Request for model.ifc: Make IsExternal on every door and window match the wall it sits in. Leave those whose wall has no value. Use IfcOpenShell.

First a look at what the model holds.

```python
import ifcopenshell
import ifcopenshell.util.element

model = ifcopenshell.open("model.ifc")
print(model.schema)
seen = {}
for e in model.by_type("IfcDoor") + model.by_type("IfcWindow"):
    if not e.FillsVoids:
        continue
    host = e.FillsVoids[0].RelatingOpeningElement.VoidsElements[0].RelatingBuildingElement
    own = ifcopenshell.util.element.get_pset(e, f"Pset_{e.is_a()[3:].removesuffix('StandardCase')}Common", "IsExternal")
    wall = ifcopenshell.util.element.get_pset(host, "Pset_WallCommon", "IsExternal")
    seen[e.is_a(), own, wall] = seen.get((e.is_a(), own, wall), 0) + 1
for (cls, own, wall), count in sorted(seen.items(), key=str):
    print(count, cls, "IsExternal:", own, "| host wall:", wall)
```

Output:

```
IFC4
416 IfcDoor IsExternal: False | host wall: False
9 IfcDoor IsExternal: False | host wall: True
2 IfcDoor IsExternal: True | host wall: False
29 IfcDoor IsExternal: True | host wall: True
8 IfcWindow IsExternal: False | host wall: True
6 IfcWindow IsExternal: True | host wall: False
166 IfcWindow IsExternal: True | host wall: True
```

```python
import ifcopenshell
import ifcopenshell.api.pset
import ifcopenshell.util.element

model = ifcopenshell.open("model.ifc")

count = 0
for ifc_class, pset_name in (("IfcDoor", "Pset_DoorCommon"), ("IfcWindow", "Pset_WindowCommon")):
    for e in model.by_type(ifc_class):
        if not e.FillsVoids:
            continue
        host = e.FillsVoids[0].RelatingOpeningElement.VoidsElements[0].RelatingBuildingElement
        external = ifcopenshell.util.element.get_pset(host, "Pset_WallCommon", "IsExternal")
        if external is None or ifcopenshell.util.element.get_pset(e, pset_name, "IsExternal") == external:
            continue
        pset = ifcopenshell.api.pset.add_pset(model, product=e, name=pset_name)
        ifcopenshell.api.pset.edit_pset(model, pset=pset, properties={"IsExternal": external})
        count += 1

print(count, "updated")

model.write("model_updated.ifc")
```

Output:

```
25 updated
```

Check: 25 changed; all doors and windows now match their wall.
